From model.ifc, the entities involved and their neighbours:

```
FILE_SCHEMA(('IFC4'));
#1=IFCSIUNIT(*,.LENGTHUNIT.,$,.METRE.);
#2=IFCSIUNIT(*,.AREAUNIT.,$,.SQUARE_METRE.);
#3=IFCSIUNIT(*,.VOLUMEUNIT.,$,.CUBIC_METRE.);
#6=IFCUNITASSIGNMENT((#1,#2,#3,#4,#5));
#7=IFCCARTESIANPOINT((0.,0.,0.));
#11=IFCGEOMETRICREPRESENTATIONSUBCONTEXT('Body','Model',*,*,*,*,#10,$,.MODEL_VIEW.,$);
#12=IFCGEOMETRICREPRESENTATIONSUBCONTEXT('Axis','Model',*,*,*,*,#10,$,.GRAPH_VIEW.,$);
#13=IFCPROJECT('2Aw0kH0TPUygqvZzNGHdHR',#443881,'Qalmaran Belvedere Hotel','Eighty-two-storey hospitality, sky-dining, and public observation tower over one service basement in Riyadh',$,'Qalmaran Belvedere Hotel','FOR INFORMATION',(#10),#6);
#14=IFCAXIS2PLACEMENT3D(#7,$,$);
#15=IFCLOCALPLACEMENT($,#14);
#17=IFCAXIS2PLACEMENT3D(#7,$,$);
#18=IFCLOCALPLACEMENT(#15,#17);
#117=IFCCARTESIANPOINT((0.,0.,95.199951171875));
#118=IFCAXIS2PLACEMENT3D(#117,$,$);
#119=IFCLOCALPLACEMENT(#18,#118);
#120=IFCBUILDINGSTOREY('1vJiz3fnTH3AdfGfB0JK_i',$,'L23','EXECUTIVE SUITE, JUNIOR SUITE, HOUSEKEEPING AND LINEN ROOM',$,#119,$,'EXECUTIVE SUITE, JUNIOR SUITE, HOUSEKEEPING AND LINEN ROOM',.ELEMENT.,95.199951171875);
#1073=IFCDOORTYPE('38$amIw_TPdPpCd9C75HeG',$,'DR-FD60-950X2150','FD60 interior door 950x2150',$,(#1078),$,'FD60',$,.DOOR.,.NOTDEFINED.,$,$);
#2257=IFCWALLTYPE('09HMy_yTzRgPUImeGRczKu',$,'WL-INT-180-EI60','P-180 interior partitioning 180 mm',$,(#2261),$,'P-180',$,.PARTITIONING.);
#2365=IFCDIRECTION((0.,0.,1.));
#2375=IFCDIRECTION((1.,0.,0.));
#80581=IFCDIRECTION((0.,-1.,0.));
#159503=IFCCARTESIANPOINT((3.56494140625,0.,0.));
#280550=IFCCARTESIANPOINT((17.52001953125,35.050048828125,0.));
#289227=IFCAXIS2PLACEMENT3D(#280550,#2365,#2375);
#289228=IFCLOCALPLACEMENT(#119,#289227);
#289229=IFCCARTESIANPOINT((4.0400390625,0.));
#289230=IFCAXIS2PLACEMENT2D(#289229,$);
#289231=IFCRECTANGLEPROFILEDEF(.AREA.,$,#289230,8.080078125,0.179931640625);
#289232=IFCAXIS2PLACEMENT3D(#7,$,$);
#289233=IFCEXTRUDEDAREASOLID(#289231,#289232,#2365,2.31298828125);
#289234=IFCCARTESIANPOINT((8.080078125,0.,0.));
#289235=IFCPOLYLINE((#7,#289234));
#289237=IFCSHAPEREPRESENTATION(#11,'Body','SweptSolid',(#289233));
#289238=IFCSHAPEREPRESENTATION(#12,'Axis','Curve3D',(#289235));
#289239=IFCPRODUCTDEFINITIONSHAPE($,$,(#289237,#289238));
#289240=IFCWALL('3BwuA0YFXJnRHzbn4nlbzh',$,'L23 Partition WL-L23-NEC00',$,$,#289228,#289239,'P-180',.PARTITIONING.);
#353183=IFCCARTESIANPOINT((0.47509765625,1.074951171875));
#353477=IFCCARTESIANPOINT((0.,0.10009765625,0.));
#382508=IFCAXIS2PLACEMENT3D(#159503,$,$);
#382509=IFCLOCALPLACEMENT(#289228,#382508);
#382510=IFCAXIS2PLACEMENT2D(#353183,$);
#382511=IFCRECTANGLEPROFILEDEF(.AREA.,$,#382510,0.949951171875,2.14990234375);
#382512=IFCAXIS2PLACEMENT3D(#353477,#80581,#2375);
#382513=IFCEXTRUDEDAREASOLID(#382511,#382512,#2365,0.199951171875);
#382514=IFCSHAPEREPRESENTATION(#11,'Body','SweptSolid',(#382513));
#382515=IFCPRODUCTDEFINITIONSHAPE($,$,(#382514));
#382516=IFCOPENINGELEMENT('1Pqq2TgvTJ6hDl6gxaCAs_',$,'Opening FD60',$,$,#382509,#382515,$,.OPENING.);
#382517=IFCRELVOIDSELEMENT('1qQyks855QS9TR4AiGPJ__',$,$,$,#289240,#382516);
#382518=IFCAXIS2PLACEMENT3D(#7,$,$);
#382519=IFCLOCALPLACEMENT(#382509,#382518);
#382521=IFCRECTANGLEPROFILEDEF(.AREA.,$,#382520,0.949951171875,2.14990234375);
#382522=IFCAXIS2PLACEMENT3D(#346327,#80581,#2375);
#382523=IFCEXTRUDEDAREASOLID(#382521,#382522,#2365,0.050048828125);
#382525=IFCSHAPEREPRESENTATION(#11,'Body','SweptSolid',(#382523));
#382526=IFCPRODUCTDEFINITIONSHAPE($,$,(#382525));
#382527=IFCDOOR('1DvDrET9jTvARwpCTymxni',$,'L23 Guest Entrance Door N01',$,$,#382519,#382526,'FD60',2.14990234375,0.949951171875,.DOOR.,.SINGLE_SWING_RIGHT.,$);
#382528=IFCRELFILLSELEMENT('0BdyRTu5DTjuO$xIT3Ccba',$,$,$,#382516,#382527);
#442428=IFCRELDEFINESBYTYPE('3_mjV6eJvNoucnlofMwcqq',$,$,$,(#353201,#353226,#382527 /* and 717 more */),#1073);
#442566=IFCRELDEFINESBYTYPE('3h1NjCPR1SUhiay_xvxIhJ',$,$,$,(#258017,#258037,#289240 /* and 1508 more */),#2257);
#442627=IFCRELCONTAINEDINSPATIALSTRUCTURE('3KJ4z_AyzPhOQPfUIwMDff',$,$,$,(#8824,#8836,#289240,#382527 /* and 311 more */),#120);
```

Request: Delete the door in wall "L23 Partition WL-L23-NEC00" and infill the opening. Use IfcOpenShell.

```python
import ifcopenshell
import ifcopenshell.api.feature
import ifcopenshell.api.root
import ifcopenshell.geom
import ifcopenshell.util.shape

model = ifcopenshell.open("model.ifc")
settings = ifcopenshell.geom.settings()


def volume(element):
    """Net volume in cubic metres, openings subtracted."""
    shape = ifcopenshell.geom.create_shape(settings, element)
    return ifcopenshell.util.shape.get_volume(shape.geometry)


door = model.by_guid("1DvDrET9jTvARwpCTymxni")
opening = door.FillsVoids[0].RelatingOpeningElement
wall = opening.VoidsElements[0].RelatingBuildingElement
before = volume(wall)

ifcopenshell.api.root.remove_product(model, product=door)
ifcopenshell.api.feature.remove_feature(model, feature=opening)

after = volume(wall)

print(f"wall volume {before:.3f} -> {after:.3f} m3")

model.write("model_v2.ifc")
```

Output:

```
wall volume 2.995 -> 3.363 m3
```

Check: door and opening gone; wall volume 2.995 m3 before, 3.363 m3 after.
